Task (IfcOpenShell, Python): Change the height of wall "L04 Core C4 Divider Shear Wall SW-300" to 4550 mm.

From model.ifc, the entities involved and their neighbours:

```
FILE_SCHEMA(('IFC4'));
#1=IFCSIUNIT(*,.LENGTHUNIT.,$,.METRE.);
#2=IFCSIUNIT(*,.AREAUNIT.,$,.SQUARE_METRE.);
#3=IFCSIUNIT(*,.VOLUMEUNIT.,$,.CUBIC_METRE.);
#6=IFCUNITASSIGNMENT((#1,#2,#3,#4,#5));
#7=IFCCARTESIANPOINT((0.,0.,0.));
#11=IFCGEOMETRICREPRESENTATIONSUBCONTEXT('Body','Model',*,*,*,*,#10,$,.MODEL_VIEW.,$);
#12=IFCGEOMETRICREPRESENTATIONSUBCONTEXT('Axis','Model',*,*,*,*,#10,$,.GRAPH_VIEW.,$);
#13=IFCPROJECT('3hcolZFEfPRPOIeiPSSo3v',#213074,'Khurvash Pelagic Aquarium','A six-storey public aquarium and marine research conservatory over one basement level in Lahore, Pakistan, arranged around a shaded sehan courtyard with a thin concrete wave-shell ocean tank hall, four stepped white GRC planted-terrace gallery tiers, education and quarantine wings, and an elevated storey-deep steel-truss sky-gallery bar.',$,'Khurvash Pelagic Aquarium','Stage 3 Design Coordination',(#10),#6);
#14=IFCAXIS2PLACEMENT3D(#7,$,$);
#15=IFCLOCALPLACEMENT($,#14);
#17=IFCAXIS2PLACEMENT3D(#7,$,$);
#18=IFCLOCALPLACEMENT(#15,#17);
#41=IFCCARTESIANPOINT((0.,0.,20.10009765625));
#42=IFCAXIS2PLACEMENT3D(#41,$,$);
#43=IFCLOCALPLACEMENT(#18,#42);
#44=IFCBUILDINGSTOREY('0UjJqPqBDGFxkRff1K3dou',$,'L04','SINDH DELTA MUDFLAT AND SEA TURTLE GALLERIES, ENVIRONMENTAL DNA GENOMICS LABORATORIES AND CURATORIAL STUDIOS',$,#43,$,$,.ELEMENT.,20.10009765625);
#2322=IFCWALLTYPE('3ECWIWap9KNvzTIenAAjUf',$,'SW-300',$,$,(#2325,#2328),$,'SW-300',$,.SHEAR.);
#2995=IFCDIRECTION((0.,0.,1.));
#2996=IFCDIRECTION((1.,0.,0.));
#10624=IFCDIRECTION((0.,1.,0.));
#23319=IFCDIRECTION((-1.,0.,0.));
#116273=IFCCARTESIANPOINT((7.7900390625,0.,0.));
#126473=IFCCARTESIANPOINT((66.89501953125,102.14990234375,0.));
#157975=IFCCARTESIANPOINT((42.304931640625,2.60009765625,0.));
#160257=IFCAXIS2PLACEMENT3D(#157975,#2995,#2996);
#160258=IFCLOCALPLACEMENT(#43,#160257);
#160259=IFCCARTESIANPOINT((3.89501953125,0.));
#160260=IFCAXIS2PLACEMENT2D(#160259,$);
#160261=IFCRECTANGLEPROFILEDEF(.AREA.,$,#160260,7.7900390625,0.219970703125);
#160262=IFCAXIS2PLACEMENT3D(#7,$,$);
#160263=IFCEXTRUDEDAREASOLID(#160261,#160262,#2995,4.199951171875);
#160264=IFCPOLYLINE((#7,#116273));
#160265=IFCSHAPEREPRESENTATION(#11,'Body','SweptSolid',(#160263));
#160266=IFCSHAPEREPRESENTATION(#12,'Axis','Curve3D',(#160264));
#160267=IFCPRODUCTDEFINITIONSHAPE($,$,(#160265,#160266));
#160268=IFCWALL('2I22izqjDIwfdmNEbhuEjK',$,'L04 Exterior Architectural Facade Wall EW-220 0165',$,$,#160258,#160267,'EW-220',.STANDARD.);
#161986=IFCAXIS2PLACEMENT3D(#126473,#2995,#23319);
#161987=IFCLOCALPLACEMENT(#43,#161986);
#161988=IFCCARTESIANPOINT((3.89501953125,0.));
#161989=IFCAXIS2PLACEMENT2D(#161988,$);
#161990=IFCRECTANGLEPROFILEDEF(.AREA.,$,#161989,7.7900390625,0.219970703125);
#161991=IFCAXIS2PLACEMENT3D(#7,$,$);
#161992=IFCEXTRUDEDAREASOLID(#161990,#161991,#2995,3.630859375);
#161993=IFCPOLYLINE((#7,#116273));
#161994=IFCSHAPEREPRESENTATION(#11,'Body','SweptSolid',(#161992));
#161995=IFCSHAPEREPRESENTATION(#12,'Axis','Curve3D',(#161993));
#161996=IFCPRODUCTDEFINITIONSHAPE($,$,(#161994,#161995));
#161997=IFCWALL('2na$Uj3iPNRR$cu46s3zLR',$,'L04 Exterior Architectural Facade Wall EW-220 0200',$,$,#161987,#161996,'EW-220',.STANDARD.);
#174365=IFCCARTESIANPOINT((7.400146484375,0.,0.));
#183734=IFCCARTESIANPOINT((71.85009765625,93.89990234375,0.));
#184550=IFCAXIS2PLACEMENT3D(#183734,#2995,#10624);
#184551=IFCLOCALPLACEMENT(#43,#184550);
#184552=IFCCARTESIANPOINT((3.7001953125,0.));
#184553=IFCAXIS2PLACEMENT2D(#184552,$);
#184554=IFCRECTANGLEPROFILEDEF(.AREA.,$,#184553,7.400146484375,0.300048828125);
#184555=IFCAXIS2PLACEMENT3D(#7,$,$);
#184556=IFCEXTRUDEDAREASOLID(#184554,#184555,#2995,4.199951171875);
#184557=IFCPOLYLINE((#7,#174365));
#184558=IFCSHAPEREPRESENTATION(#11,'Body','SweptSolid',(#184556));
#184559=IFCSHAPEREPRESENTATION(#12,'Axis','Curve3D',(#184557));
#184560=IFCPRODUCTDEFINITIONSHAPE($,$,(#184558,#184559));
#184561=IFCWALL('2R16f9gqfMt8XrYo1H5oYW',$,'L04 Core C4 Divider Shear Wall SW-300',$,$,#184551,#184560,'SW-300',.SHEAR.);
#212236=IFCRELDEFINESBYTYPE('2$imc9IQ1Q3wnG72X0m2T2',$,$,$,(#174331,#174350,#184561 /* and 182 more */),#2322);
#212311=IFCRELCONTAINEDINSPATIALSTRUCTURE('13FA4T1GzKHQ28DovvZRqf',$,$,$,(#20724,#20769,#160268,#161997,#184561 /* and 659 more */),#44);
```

```python
import ifcopenshell
import ifcopenshell.geom
import ifcopenshell.util.representation
import ifcopenshell.util.shape

model = ifcopenshell.open("model.ifc")
settings = ifcopenshell.geom.settings()


def volume(element):
    """Net volume in cubic metres, openings subtracted."""
    shape = ifcopenshell.geom.create_shape(settings, element)
    return ifcopenshell.util.shape.get_volume(shape.geometry)


wall = model.by_guid("2R16f9gqfMt8XrYo1H5oYW")
before = volume(wall)

body = ifcopenshell.util.representation.get_representation(wall, "Model", "Body")
solid = body.Items[0]
old_height = solid.Depth
solid.Depth = 4.55
after = volume(wall)

print(f"height {old_height:g} -> {solid.Depth:g}, volume {before:.3f} -> {after:.3f} m3")

model.write("model_edited.ifc")
```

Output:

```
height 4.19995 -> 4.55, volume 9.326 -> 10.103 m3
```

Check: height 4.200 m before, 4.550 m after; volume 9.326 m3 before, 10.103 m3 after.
